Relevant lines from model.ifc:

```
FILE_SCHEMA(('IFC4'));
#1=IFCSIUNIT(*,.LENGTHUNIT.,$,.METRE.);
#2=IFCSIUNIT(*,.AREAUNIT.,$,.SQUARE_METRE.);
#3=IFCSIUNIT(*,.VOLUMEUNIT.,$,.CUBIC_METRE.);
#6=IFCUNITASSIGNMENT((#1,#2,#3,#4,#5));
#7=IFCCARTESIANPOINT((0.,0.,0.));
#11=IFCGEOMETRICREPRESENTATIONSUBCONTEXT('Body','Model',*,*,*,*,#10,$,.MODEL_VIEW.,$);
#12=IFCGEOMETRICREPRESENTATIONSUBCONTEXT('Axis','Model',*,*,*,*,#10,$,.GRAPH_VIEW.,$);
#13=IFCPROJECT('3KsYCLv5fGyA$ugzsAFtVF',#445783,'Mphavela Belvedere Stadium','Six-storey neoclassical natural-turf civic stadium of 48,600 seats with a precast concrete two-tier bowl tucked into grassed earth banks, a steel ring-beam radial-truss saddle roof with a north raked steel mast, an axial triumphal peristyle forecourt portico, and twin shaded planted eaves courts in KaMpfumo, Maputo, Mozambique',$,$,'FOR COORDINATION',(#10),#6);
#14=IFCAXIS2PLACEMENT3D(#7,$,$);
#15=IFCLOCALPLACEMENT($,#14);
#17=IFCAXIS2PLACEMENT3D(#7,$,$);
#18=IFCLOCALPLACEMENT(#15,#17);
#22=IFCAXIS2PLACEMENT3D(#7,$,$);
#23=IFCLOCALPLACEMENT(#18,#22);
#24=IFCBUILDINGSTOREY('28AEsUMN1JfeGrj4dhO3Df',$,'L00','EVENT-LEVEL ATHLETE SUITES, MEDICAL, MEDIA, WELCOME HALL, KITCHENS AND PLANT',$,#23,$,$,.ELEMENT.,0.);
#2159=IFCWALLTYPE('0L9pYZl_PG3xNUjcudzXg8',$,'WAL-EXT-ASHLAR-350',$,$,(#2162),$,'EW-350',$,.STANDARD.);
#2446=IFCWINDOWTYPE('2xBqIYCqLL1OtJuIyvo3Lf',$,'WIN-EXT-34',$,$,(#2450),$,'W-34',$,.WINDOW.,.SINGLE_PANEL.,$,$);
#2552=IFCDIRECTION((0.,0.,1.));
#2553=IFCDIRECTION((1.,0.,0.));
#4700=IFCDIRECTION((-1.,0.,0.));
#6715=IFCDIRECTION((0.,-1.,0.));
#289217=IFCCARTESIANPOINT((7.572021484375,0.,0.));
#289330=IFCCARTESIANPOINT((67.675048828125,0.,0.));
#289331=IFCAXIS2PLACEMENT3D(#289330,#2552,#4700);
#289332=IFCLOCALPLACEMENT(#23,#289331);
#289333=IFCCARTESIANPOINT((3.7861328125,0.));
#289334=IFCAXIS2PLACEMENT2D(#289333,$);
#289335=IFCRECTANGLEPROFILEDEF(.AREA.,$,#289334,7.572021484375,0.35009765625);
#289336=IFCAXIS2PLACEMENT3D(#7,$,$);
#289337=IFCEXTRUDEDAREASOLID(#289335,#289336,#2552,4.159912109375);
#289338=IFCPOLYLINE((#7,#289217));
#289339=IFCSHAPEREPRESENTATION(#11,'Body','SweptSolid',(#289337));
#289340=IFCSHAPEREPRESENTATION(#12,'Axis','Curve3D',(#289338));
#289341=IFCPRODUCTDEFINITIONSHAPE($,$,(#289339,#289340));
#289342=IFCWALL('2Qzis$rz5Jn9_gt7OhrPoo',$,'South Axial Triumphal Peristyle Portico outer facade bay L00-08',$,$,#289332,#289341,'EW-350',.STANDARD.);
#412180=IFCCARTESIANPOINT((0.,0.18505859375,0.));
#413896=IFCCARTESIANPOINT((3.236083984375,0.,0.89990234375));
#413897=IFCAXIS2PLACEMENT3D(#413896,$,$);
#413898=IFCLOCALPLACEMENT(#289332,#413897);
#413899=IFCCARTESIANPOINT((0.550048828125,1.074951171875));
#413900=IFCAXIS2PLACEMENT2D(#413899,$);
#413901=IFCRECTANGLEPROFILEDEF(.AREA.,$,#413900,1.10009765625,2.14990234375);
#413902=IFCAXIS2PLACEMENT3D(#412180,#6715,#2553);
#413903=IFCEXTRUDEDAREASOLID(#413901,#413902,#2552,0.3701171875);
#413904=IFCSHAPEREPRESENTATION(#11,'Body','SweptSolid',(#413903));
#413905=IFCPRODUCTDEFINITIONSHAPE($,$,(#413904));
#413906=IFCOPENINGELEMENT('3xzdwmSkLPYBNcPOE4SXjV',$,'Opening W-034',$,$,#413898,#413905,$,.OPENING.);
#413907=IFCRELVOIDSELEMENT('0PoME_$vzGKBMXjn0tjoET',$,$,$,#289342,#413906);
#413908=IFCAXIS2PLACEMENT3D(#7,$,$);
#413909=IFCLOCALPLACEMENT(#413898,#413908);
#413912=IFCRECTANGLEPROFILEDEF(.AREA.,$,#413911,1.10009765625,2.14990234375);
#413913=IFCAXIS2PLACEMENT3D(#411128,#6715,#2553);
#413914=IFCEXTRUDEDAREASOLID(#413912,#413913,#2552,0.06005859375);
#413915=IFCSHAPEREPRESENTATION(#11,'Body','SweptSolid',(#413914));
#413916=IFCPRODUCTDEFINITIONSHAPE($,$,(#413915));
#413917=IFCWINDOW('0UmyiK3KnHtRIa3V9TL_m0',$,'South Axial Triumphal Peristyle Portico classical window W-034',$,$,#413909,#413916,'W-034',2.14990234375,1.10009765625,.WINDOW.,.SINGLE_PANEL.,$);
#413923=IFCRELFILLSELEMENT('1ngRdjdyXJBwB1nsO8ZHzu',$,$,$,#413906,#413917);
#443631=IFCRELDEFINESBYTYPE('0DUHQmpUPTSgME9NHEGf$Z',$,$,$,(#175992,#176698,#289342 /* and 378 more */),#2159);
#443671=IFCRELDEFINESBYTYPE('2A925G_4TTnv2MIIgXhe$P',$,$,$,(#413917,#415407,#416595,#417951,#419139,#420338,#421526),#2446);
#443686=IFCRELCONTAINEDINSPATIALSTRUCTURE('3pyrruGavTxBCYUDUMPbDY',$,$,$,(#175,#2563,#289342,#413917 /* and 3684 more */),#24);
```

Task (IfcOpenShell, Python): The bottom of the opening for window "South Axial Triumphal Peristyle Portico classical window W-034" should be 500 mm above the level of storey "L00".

```python
import numpy as np
import ifcopenshell
import ifcopenshell.api.geometry
import ifcopenshell.geom
import ifcopenshell.util.element
import ifcopenshell.util.placement
import ifcopenshell.util.shape
import ifcopenshell.util.unit

model = ifcopenshell.open("model.ifc")
unit_scale = ifcopenshell.util.unit.calculate_unit_scale(model)

window = model.by_guid("0UmyiK3KnHtRIa3V9TL_m0")
opening = window.FillsVoids[0].RelatingOpeningElement
storey = ifcopenshell.util.element.get_container(window, ifc_class="IfcBuildingStorey")
level = ifcopenshell.util.placement.get_local_placement(storey.ObjectPlacement)[2, 3]

# The opening's origin need not be at the sill, so measure its lowest point.
shape = ifcopenshell.geom.create_shape(ifcopenshell.geom.settings(), opening)
bottom = ifcopenshell.util.shape.get_shape_bottom_elevation(shape, shape.geometry) / unit_scale
dz = level + 0.5 - bottom

shift = np.array([0.0, 0.0, dz])
# The window is placed relative to its opening, so it follows when the opening moves.
matrix = ifcopenshell.util.placement.get_local_placement(opening.ObjectPlacement)
matrix[:3, 3] += shift
ifcopenshell.api.geometry.edit_object_placement(
    model, product=opening, matrix=matrix, is_si=False, should_transform_children=True
)

print(f"moved by {dz * unit_scale:+.3f} m")

model.write("model_updated.ifc")
```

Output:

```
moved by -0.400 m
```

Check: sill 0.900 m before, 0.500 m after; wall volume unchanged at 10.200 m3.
